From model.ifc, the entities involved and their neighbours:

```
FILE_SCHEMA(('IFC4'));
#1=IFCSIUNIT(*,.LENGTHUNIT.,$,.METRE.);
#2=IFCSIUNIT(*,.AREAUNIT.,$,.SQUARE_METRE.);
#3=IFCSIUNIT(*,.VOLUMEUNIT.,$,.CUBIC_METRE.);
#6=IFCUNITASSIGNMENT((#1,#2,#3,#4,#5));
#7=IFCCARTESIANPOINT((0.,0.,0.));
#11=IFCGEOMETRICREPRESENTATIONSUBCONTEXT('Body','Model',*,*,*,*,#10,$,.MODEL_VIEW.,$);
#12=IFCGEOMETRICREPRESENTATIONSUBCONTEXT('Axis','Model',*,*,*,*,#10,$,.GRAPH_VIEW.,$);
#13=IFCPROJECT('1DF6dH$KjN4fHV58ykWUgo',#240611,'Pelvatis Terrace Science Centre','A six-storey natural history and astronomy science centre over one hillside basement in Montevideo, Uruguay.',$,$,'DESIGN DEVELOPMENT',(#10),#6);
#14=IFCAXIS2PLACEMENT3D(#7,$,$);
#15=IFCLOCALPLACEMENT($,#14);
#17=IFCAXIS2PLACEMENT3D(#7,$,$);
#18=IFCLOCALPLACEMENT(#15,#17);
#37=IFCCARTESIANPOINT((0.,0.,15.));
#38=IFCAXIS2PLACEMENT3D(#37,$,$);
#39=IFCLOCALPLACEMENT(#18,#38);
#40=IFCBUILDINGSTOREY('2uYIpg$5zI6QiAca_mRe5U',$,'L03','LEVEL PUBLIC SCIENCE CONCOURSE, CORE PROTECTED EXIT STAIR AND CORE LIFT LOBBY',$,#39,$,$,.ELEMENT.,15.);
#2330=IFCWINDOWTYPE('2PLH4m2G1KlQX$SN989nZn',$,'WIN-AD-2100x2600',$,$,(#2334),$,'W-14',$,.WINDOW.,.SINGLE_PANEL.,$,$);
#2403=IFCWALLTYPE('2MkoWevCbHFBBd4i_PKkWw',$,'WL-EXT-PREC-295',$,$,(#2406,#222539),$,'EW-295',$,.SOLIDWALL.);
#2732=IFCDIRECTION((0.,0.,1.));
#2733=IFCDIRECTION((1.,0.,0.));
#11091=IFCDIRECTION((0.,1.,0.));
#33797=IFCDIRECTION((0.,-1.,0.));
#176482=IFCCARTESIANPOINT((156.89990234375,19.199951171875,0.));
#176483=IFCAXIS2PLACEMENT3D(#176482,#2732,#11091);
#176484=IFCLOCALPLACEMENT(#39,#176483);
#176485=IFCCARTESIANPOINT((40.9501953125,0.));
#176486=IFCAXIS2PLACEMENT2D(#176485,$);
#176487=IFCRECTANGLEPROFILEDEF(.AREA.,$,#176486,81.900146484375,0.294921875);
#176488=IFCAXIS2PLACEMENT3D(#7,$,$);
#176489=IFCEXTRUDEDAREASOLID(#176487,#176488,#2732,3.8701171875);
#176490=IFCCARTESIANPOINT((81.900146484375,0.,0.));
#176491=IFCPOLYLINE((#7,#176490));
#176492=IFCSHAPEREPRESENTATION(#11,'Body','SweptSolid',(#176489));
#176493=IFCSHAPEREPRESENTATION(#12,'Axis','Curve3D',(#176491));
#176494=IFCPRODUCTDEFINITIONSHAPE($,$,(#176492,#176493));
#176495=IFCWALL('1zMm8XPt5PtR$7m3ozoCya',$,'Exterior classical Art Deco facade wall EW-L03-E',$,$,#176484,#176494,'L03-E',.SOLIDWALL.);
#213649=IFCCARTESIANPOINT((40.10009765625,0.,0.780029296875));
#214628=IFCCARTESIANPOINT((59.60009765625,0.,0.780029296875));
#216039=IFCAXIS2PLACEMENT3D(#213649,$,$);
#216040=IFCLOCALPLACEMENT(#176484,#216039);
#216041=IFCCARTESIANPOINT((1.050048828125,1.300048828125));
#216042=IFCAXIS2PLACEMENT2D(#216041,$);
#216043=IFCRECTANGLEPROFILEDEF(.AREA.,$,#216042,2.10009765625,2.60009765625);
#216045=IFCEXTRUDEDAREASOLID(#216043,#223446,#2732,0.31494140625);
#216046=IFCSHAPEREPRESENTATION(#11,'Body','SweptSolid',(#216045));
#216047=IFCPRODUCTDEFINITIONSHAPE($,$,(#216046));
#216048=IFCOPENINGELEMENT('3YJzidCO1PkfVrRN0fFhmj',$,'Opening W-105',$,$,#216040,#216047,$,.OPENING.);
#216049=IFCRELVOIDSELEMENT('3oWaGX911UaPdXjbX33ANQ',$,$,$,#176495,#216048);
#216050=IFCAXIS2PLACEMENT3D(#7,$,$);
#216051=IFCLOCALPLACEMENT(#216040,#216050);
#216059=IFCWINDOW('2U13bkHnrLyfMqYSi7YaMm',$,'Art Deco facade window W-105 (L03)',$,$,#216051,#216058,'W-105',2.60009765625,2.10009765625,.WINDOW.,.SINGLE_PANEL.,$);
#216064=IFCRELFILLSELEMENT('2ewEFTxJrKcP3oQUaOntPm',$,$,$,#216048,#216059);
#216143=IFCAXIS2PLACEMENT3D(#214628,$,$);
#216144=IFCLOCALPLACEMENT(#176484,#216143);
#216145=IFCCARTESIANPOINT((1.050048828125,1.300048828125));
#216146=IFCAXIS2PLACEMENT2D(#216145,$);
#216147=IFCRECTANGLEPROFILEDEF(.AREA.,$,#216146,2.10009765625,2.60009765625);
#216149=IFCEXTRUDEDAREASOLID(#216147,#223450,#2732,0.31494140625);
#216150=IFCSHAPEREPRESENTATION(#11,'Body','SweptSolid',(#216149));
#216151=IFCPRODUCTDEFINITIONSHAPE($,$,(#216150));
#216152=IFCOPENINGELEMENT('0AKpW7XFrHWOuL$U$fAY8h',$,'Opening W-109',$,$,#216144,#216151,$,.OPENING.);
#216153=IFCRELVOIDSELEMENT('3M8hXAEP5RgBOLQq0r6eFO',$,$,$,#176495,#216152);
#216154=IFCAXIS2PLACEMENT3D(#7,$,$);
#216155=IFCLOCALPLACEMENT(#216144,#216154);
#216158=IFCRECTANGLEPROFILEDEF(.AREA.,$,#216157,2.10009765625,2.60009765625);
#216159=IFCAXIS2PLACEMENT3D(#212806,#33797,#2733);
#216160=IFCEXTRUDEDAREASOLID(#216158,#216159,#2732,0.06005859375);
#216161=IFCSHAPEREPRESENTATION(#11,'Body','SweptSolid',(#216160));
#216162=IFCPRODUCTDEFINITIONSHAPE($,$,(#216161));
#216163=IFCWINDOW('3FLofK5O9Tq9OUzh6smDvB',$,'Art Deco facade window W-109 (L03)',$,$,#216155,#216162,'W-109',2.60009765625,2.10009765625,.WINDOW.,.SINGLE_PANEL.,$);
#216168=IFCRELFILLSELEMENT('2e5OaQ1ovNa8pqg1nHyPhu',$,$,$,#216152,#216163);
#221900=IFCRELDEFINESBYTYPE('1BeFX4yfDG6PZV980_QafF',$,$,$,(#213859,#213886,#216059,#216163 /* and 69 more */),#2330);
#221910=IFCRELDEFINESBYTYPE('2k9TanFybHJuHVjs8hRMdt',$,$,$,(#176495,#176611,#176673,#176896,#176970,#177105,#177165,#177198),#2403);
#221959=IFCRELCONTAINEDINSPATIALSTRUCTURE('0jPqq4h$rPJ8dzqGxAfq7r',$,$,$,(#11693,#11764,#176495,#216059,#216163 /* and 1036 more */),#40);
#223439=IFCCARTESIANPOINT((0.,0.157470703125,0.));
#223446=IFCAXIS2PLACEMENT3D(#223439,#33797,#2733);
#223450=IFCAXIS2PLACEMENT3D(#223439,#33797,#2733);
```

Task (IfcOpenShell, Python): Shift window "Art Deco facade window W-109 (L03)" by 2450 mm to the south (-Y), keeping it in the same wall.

```python
import ifcopenshell
import ifcopenshell.api.geometry
import ifcopenshell.util.placement
import ifcopenshell.util.unit

model = ifcopenshell.open("model.ifc")
unit_scale = ifcopenshell.util.unit.calculate_unit_scale(model)

window = model.by_guid("3FLofK5O9Tq9OUzh6smDvB")
opening = window.FillsVoids[0].RelatingOpeningElement
wall = opening.VoidsElements[0].RelatingBuildingElement

wall_matrix = ifcopenshell.util.placement.get_local_placement(wall.ObjectPlacement)
shift = wall_matrix[:3, 0] * -2.45 / unit_scale
before = ifcopenshell.util.placement.get_local_placement(window.ObjectPlacement)[:3, 3].copy()

# The window is placed relative to its opening, so it follows when the opening moves.
matrix = ifcopenshell.util.placement.get_local_placement(opening.ObjectPlacement)
matrix[:3, 3] += shift
ifcopenshell.api.geometry.edit_object_placement(
    model, product=opening, matrix=matrix, is_si=False, should_transform_children=True
)

after = ifcopenshell.util.placement.get_local_placement(window.ObjectPlacement)[:3, 3]
print("window moved by", (after - before).round(3) + 0.0)

model.write("model_rev.ifc")
```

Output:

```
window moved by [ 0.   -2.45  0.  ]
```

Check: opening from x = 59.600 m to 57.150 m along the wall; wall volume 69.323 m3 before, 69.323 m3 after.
